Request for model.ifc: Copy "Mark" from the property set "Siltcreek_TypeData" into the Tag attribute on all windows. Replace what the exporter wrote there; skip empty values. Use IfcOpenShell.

First a look at what the model holds.

```python
import ifcopenshell
import ifcopenshell.util.element

model = ifcopenshell.open("model.ifc")
print(model.schema)
windows = model.by_type("IfcWindow")
print(len(windows), "windows")
for e in windows[:8]:
    source = ifcopenshell.util.element.get_pset(e, "Siltcreek_TypeData", "Mark")
    target = e.Tag
    print(e.id(), repr(source), repr(target), sep=" | ")
```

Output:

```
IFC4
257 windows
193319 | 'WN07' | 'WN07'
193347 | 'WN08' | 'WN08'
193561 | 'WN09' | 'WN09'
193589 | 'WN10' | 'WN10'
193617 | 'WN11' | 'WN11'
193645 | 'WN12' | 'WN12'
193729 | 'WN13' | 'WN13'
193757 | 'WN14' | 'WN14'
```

```python
import ifcopenshell
import ifcopenshell.util.element

model = ifcopenshell.open("model.ifc")

count = 0
for e in model.by_type("IfcWindow"):
    value = ifcopenshell.util.element.get_pset(e, "Siltcreek_TypeData", "Mark")
    current = e.Tag
    if not value or not value.strip() or current == value:
        continue
    e.Tag = value
    count += 1

print(count, "windows updated")

model.write("model-out.ifc")
```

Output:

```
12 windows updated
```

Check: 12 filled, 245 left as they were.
